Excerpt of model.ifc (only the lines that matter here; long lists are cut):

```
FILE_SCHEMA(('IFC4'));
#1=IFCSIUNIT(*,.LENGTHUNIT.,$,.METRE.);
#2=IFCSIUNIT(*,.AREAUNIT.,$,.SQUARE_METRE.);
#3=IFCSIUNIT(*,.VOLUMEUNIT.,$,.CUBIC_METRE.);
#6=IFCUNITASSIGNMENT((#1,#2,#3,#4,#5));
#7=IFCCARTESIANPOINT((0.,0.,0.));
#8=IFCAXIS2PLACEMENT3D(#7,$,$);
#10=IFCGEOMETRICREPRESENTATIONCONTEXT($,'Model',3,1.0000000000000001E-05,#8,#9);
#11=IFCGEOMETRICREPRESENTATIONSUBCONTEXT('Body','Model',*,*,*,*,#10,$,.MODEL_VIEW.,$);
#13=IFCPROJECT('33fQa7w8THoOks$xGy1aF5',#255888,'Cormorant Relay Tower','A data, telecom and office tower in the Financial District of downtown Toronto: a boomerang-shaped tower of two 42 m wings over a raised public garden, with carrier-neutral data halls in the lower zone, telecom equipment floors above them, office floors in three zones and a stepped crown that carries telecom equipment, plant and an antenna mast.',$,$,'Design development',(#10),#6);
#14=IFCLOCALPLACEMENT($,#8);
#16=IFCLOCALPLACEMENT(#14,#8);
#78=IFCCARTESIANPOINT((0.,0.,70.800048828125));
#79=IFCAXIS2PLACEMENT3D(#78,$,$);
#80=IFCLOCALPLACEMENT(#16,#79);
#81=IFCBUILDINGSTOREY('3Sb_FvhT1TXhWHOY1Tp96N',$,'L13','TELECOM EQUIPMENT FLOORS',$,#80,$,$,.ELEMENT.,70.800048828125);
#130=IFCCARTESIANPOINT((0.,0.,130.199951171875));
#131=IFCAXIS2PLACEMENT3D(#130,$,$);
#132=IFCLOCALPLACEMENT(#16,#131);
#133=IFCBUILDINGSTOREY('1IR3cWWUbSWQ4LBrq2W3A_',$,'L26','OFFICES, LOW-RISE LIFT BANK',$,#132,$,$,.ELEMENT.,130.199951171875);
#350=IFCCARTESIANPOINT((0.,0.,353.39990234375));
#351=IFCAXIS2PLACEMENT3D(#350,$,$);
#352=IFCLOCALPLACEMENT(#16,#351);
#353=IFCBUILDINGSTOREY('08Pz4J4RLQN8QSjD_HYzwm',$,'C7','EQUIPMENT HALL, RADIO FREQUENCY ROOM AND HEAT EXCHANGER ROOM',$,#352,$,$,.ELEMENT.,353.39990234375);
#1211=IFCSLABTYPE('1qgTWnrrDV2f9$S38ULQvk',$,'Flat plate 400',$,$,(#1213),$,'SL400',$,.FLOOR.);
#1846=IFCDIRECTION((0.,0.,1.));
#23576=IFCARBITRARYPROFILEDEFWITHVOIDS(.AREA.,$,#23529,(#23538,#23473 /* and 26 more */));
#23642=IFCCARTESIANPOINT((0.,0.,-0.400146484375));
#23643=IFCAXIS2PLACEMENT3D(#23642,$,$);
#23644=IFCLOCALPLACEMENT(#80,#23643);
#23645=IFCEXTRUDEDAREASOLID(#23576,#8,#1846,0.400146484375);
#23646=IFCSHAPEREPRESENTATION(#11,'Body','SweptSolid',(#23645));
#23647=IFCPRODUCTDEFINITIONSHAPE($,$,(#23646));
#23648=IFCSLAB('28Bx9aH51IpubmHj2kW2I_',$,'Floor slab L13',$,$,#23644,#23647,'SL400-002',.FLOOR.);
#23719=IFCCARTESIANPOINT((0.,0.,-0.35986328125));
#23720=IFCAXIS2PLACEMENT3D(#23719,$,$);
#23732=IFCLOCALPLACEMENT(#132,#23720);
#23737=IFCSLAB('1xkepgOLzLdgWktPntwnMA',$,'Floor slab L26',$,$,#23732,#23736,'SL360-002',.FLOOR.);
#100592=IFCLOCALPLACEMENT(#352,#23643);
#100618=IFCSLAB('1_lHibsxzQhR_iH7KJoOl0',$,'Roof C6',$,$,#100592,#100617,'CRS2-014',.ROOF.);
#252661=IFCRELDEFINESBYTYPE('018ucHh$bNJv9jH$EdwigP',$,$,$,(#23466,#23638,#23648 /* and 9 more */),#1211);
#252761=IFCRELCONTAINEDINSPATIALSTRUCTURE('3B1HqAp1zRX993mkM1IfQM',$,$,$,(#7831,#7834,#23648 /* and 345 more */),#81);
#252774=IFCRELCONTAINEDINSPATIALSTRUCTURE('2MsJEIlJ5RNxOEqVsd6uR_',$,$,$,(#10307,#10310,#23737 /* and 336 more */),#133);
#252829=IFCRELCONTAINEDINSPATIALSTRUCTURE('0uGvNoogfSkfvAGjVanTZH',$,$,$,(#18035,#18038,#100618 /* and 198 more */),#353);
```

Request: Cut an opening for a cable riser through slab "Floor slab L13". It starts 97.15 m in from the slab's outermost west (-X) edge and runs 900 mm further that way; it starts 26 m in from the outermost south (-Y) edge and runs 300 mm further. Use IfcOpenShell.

```python
import numpy as np
import ifcopenshell
import ifcopenshell.api.feature
import ifcopenshell.api.geometry
import ifcopenshell.api.root
import ifcopenshell.geom
import ifcopenshell.util.placement
import ifcopenshell.util.representation
import ifcopenshell.util.shape
import ifcopenshell.util.unit

model = ifcopenshell.open("model.ifc")
unit_scale = ifcopenshell.util.unit.calculate_unit_scale(model)
settings = ifcopenshell.geom.settings()


def volume(element):
    """Net volume in cubic metres, openings subtracted."""
    shape = ifcopenshell.geom.create_shape(settings, element)
    return ifcopenshell.util.shape.get_volume(shape.geometry)


slab = model.by_id(23648)
before = volume(slab)

# Extent in the slab's own axes, in metres. The edges named are its -X and -Y sides.
slab_shape = ifcopenshell.geom.create_shape(settings, slab)
vertices = ifcopenshell.util.shape.get_vertices(slab_shape.geometry)
x_min, y_min, bottom = vertices.min(axis=0)
top = vertices[:, 2].max()

opening = ifcopenshell.api.root.create_entity(model, ifc_class="IfcOpeningElement", name="Cable riser opening", predefined_type="OPENING")
context = ifcopenshell.util.representation.get_context(model, "Model", "Body", "MODEL_VIEW")
width, depth = 0.9, 0.3
outline = [(0.0, 0.0), (width, 0.0), (width, depth), (0.0, depth), (0.0, 0.0)]
# Overshoot both faces by 50 mm so the cut is clean.
shape = ifcopenshell.api.geometry.add_slab_representation(
    model, context=context, depth=top - bottom + 0.1, polyline=outline
)
ifcopenshell.api.geometry.assign_representation(model, product=opening, representation=shape)

matrix = ifcopenshell.util.placement.get_local_placement(slab.ObjectPlacement)
matrix[:, 3] = matrix @ np.append(np.array([x_min + 97.15, y_min + 26, bottom - 0.05]) / unit_scale, 1.0)
ifcopenshell.api.geometry.edit_object_placement(model, product=opening, matrix=matrix, is_si=False)
ifcopenshell.api.feature.add_feature(model, feature=opening, element=slab)

after = volume(slab)

print(f"slab volume {before:.3f} -> {after:.3f} m3")

model.write("model_rev.ifc")
```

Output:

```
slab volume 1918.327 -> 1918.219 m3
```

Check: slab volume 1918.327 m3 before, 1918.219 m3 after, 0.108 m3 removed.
